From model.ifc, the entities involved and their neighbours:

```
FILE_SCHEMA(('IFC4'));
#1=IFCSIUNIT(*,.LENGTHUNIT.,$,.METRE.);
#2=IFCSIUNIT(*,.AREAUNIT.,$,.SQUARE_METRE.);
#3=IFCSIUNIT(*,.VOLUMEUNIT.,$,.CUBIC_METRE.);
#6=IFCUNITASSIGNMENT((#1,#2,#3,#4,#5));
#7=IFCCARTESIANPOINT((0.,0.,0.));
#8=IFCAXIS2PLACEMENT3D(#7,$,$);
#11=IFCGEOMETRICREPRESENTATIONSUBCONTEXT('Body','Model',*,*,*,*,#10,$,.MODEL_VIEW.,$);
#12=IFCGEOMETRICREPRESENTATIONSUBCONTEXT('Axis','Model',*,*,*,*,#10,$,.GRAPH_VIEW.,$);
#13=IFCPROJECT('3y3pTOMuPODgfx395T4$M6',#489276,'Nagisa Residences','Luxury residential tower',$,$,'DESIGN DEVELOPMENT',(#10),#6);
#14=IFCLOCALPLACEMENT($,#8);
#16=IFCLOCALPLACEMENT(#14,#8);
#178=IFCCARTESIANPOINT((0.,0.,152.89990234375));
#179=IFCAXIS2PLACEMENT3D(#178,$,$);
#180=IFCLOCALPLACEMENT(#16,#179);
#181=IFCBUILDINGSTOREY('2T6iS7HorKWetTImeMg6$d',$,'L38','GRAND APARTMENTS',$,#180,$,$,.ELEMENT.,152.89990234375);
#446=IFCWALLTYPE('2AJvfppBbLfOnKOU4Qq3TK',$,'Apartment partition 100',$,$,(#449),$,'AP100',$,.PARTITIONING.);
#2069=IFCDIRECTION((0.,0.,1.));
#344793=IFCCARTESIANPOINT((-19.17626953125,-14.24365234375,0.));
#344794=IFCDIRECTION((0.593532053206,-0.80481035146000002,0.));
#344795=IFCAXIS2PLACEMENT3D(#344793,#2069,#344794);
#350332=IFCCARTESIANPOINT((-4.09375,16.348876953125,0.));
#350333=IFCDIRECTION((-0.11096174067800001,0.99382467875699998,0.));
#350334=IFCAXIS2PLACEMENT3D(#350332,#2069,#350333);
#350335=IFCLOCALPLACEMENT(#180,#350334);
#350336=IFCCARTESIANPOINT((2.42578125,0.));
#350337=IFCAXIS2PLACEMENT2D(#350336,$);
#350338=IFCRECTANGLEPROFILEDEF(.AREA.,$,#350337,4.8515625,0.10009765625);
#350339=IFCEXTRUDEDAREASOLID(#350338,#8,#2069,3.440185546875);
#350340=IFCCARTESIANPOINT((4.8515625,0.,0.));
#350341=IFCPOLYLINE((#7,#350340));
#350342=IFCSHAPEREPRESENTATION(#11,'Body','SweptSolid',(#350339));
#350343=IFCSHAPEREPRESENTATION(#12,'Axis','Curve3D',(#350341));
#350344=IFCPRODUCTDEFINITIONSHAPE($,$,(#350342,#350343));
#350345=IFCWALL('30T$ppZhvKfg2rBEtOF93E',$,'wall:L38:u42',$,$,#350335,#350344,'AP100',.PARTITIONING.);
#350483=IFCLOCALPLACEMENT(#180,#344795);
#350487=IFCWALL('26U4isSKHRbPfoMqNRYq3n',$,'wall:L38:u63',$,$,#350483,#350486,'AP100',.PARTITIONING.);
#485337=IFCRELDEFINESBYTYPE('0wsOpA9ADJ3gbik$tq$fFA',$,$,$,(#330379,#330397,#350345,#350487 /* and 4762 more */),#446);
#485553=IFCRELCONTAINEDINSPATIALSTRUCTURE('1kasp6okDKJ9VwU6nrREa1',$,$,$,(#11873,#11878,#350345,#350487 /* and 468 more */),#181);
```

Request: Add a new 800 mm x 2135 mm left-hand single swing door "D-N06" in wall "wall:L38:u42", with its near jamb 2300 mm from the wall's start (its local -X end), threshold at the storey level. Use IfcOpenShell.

```python
import numpy as np
import ifcopenshell
import ifcopenshell.api.feature
import ifcopenshell.api.geometry
import ifcopenshell.api.root
import ifcopenshell.api.spatial
import ifcopenshell.geom
import ifcopenshell.util.element
import ifcopenshell.util.placement
import ifcopenshell.util.representation
import ifcopenshell.util.shape
import ifcopenshell.util.unit

model = ifcopenshell.open("model.ifc")
unit_scale = ifcopenshell.util.unit.calculate_unit_scale(model)
settings = ifcopenshell.geom.settings()


def volume(element):
    """Net volume in cubic metres, openings subtracted."""
    shape = ifcopenshell.geom.create_shape(settings, element)
    return ifcopenshell.util.shape.get_volume(shape.geometry)


wall = model.by_guid("30T$ppZhvKfg2rBEtOF93E")
storey = ifcopenshell.util.element.get_container(wall, ifc_class="IfcBuildingStorey")
context = ifcopenshell.util.representation.get_context(model, "Model", "Body", "MODEL_VIEW")
before = volume(wall)

width, height, from_end, sill = 0.8, 2.135, 2.3, 0.0  # metres

# The wall runs along its own X axis, and the end named is its -X end.
wall_shape = ifcopenshell.geom.create_shape(settings, wall)
x, y, z = ifcopenshell.util.shape.get_vertices(wall_shape.geometry).T
start = x.min() + from_end
face, thickness = float(y.min()), float(y.max() - y.min())
wall_matrix = ifcopenshell.util.placement.get_local_placement(wall.ObjectPlacement)
level = ifcopenshell.util.placement.get_local_placement(storey.ObjectPlacement)[2, 3]


def in_wall(x, y):
    """Placement at x, y metres in the wall's axes, at sill height."""
    matrix = wall_matrix.copy()
    matrix[:, 3] = wall_matrix @ np.array([x / unit_scale, y / unit_scale, 0.0, 1.0])
    matrix[2, 3] = level + sill / unit_scale
    return matrix


# Opening: a box that overshoots both wall faces by 50 mm.
opening = ifcopenshell.api.root.create_entity(model, ifc_class="IfcOpeningElement", predefined_type="OPENING")
box = ifcopenshell.api.geometry.add_wall_representation(
    model, context=context, length=width, height=height, thickness=thickness + 0.1
)
ifcopenshell.api.geometry.assign_representation(model, product=opening, representation=box)
ifcopenshell.api.geometry.edit_object_placement(model, product=opening, matrix=in_wall(start, face - 0.05), is_si=False)
ifcopenshell.api.feature.add_feature(model, feature=opening, element=wall)

door = ifcopenshell.api.root.create_entity(model, ifc_class="IfcDoor", name="D-N06", predefined_type="DOOR")
door.OverallWidth, door.OverallHeight = width / unit_scale, height / unit_scale
door.OperationType = "SINGLE_SWING_LEFT"
body = ifcopenshell.api.geometry.add_door_representation(
    model,
    context=context,
    overall_width=door.OverallWidth,
    overall_height=door.OverallHeight,
    operation_type="SINGLE_SWING_LEFT",
    lining_properties={"LiningDepth": thickness / unit_scale, "ThresholdDepth": thickness / unit_scale},
)
ifcopenshell.api.geometry.assign_representation(model, product=door, representation=body)
ifcopenshell.api.spatial.assign_container(model, products=[door], relating_structure=storey)
ifcopenshell.api.feature.add_filling(model, opening=opening, element=door)

# The lining spans the wall, so the door starts at the wall face.
ifcopenshell.api.geometry.edit_object_placement(model, product=door, matrix=in_wall(start, face), is_si=False)

after = volume(wall)

print(f"wall volume {before:.3f} -> {after:.3f} m3")

model.write("model-out.ifc")
```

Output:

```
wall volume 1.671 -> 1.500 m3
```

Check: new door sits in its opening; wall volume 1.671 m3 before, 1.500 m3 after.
